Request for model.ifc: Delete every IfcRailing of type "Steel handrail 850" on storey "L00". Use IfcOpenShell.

First a look at what the model holds.

```python
import ifcopenshell
import ifcopenshell.util.element

model = ifcopenshell.open("model.ifc")
print(model.schema)
storey = next(s for s in model.by_type("IfcBuildingStorey") if s.Name == "L00")
railings = [e for e in ifcopenshell.util.element.get_decomposition(storey) if e.is_a("IfcRailing")]
seen = {}
for e in railings:
    element_type = ifcopenshell.util.element.get_type(e)
    name = element_type.Name if element_type not in (None, e) else None
    seen[name] = seen.get(name, 0) + 1
for name, count in sorted(seen.items(), key=str):
    print(count, "x", name)
```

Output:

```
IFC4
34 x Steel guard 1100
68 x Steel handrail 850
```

```python
import ifcopenshell
import ifcopenshell.api.root
import ifcopenshell.util.element

model = ifcopenshell.open("model.ifc")

storey = next(s for s in model.by_type("IfcBuildingStorey") if s.Name == "L00")
railings = [e for e in ifcopenshell.util.element.get_decomposition(storey) if e.is_a("IfcRailing")]
targets = [e for e in railings if (t := ifcopenshell.util.element.get_type(e)) not in (None, e) and t.Name == "Steel handrail 850"]

for e in targets:
    ifcopenshell.api.root.remove_product(model, product=e)
print(len(targets), "removed")

model.write("model_v2.ifc")
```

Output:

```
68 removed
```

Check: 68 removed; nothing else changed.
